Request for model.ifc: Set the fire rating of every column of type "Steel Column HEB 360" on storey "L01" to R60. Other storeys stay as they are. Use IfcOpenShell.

First a look at what the model holds.

```python
import ifcopenshell
import ifcopenshell.util.element

model = ifcopenshell.open("model.ifc")
print(model.schema)
storey = next(s for s in model.by_type("IfcBuildingStorey") if s.Name == "L01")
columns = [e for e in ifcopenshell.util.element.get_decomposition(storey) if e.is_a("IfcColumn")]
seen = {}
for e in columns:
    element_type = ifcopenshell.util.element.get_type(e)
    key = (element_type.Name if element_type != e and element_type else None, ifcopenshell.util.element.get_pset(e, "Pset_ColumnCommon", "FireRating"))
    seen[key] = seen.get(key, 0) + 1
for (name, value), count in sorted(seen.items(), key=str):
    print(count, "x", name, "|", value)
```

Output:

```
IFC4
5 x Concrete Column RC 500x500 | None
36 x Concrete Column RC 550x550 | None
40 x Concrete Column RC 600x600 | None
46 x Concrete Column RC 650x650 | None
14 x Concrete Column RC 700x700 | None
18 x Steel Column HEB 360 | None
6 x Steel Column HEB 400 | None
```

```python
import ifcopenshell
import ifcopenshell.api.pset
import ifcopenshell.util.element

model = ifcopenshell.open("model.ifc")

storey = next(s for s in model.by_type("IfcBuildingStorey") if s.Name == "L01")
columns = [e for e in ifcopenshell.util.element.get_decomposition(storey) if e.is_a("IfcColumn")]

count = 0
for e in columns:
    element_type = ifcopenshell.util.element.get_type(e)
    if element_type in (None, e) or element_type.Name != "Steel Column HEB 360":
        continue
    # add_pset returns the element's existing set when there is one.
    pset = ifcopenshell.api.pset.add_pset(model, product=e, name="Pset_ColumnCommon")
    ifcopenshell.api.pset.edit_pset(model, pset=pset, properties={"FireRating": "R60"})
    count += 1

print(count, "columns updated")

model.write("model-out.ifc")
```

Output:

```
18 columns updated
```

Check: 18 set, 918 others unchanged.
